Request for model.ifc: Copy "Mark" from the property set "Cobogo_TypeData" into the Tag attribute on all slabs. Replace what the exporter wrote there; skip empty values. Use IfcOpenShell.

First a look at what the model holds.

```python
import ifcopenshell
import ifcopenshell.util.element

model = ifcopenshell.open("model.ifc")
print(model.schema)
slabs = model.by_type("IfcSlab")
print(len(slabs), "slabs")
for e in slabs[:8]:
    source = ifcopenshell.util.element.get_pset(e, "Cobogo_TypeData", "Mark")
    target = e.Tag
    print(e.id(), repr(source), repr(target), sep=" | ")
```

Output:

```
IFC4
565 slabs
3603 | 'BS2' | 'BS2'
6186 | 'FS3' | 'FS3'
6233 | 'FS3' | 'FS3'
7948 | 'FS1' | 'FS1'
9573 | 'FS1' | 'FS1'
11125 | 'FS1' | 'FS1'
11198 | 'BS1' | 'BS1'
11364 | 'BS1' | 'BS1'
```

```python
import ifcopenshell
import ifcopenshell.util.element

model = ifcopenshell.open("model.ifc")

count = 0
for e in model.by_type("IfcSlab"):
    value = ifcopenshell.util.element.get_pset(e, "Cobogo_TypeData", "Mark")
    current = e.Tag
    if not value or not value.strip() or current == value:
        continue
    e.Tag = value
    count += 1

print(count, "slabs updated")

model.write("model_updated.ifc")
```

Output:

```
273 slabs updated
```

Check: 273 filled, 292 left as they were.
